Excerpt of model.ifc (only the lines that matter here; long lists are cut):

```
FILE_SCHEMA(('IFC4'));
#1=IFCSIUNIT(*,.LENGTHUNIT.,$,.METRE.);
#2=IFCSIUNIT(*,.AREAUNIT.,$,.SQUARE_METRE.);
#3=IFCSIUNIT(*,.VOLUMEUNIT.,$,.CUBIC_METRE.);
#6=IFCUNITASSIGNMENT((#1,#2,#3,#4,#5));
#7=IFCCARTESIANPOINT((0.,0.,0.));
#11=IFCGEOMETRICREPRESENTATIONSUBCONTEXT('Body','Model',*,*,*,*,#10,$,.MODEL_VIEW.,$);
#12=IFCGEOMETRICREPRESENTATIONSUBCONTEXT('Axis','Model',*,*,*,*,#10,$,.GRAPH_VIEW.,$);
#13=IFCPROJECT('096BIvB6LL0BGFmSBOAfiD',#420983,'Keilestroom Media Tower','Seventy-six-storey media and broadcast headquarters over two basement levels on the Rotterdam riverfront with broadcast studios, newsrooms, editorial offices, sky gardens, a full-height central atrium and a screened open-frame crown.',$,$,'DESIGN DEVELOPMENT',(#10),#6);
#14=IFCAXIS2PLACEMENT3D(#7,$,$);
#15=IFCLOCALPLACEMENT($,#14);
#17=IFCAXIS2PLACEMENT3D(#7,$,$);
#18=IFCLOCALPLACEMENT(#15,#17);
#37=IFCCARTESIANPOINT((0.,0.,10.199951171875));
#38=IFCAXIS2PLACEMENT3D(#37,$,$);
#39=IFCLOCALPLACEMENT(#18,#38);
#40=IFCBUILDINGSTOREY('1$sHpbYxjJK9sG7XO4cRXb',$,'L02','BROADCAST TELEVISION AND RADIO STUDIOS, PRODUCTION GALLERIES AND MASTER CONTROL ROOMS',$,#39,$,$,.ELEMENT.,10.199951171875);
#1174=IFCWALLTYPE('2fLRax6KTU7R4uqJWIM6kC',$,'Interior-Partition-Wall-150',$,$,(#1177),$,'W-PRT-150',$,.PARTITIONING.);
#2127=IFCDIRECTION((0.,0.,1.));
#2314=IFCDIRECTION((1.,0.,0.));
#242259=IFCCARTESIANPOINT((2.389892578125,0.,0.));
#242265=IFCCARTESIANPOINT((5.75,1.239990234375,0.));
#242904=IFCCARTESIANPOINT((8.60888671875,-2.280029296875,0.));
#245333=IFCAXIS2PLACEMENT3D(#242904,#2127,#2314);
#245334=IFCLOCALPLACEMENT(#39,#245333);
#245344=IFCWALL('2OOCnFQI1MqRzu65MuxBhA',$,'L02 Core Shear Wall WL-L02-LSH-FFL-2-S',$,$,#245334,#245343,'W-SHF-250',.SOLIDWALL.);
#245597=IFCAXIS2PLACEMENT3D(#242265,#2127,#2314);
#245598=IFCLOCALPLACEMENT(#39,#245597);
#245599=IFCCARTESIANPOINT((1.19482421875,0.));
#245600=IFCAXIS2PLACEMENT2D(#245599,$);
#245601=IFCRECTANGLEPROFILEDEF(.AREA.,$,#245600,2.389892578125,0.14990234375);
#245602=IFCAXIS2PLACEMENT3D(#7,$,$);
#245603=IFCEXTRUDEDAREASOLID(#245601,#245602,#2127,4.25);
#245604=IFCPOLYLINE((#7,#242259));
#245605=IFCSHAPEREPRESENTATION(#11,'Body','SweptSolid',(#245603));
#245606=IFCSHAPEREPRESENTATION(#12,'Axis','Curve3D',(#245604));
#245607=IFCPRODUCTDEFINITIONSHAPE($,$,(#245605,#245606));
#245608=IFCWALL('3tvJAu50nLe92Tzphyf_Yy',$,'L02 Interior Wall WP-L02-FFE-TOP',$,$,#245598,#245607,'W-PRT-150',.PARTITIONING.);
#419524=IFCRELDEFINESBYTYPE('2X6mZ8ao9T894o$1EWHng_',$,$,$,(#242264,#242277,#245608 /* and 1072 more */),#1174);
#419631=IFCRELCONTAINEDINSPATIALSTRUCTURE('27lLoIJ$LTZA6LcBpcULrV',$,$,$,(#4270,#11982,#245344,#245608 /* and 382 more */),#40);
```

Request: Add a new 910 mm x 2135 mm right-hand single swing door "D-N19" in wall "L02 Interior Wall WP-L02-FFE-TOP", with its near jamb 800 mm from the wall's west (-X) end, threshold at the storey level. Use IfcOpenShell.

```python
import numpy as np
import ifcopenshell
import ifcopenshell.api.feature
import ifcopenshell.api.geometry
import ifcopenshell.api.root
import ifcopenshell.api.spatial
import ifcopenshell.geom
import ifcopenshell.util.element
import ifcopenshell.util.placement
import ifcopenshell.util.representation
import ifcopenshell.util.shape
import ifcopenshell.util.unit

model = ifcopenshell.open("model.ifc")
unit_scale = ifcopenshell.util.unit.calculate_unit_scale(model)
settings = ifcopenshell.geom.settings()


def volume(element):
    """Net volume in cubic metres, openings subtracted."""
    shape = ifcopenshell.geom.create_shape(settings, element)
    return ifcopenshell.util.shape.get_volume(shape.geometry)


wall = model.by_id(245608)
storey = ifcopenshell.util.element.get_container(wall, ifc_class="IfcBuildingStorey")
context = ifcopenshell.util.representation.get_context(model, "Model", "Body", "MODEL_VIEW")
before = volume(wall)

width, height, from_end, sill = 0.91, 2.135, 0.8, 0.0  # metres

# The wall runs along its own X axis, and the end named is its -X end.
wall_shape = ifcopenshell.geom.create_shape(settings, wall)
x, y, z = ifcopenshell.util.shape.get_vertices(wall_shape.geometry).T
start = x.min() + from_end
face, thickness = float(y.min()), float(y.max() - y.min())
wall_matrix = ifcopenshell.util.placement.get_local_placement(wall.ObjectPlacement)
level = ifcopenshell.util.placement.get_local_placement(storey.ObjectPlacement)[2, 3]


def in_wall(x, y):
    """Placement at x, y metres in the wall's axes, at sill height."""
    matrix = wall_matrix.copy()
    matrix[:, 3] = wall_matrix @ np.array([x / unit_scale, y / unit_scale, 0.0, 1.0])
    matrix[2, 3] = level + sill / unit_scale
    return matrix


# Opening: a box that overshoots both wall faces by 50 mm.
opening = ifcopenshell.api.root.create_entity(model, ifc_class="IfcOpeningElement", predefined_type="OPENING")
box = ifcopenshell.api.geometry.add_wall_representation(
    model, context=context, length=width, height=height, thickness=thickness + 0.1
)
ifcopenshell.api.geometry.assign_representation(model, product=opening, representation=box)
ifcopenshell.api.geometry.edit_object_placement(model, product=opening, matrix=in_wall(start, face - 0.05), is_si=False)
ifcopenshell.api.feature.add_feature(model, feature=opening, element=wall)

door = ifcopenshell.api.root.create_entity(model, ifc_class="IfcDoor", name="D-N19", predefined_type="DOOR")
door.OverallWidth, door.OverallHeight = width / unit_scale, height / unit_scale
door.OperationType = "SINGLE_SWING_RIGHT"
body = ifcopenshell.api.geometry.add_door_representation(
    model,
    context=context,
    overall_width=door.OverallWidth,
    overall_height=door.OverallHeight,
    operation_type="SINGLE_SWING_RIGHT",
    lining_properties={"LiningDepth": thickness / unit_scale, "ThresholdDepth": thickness / unit_scale},
)
ifcopenshell.api.geometry.assign_representation(model, product=door, representation=body)
ifcopenshell.api.spatial.assign_container(model, products=[door], relating_structure=storey)
ifcopenshell.api.feature.add_filling(model, opening=opening, element=door)

# The lining spans the wall, so the door starts at the wall face.
ifcopenshell.api.geometry.edit_object_placement(model, product=door, matrix=in_wall(start, face), is_si=False)

after = volume(wall)

print(f"wall volume {before:.3f} -> {after:.3f} m3")

model.write("model_edited.ifc")
```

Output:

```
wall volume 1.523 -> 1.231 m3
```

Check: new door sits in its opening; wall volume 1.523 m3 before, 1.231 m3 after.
